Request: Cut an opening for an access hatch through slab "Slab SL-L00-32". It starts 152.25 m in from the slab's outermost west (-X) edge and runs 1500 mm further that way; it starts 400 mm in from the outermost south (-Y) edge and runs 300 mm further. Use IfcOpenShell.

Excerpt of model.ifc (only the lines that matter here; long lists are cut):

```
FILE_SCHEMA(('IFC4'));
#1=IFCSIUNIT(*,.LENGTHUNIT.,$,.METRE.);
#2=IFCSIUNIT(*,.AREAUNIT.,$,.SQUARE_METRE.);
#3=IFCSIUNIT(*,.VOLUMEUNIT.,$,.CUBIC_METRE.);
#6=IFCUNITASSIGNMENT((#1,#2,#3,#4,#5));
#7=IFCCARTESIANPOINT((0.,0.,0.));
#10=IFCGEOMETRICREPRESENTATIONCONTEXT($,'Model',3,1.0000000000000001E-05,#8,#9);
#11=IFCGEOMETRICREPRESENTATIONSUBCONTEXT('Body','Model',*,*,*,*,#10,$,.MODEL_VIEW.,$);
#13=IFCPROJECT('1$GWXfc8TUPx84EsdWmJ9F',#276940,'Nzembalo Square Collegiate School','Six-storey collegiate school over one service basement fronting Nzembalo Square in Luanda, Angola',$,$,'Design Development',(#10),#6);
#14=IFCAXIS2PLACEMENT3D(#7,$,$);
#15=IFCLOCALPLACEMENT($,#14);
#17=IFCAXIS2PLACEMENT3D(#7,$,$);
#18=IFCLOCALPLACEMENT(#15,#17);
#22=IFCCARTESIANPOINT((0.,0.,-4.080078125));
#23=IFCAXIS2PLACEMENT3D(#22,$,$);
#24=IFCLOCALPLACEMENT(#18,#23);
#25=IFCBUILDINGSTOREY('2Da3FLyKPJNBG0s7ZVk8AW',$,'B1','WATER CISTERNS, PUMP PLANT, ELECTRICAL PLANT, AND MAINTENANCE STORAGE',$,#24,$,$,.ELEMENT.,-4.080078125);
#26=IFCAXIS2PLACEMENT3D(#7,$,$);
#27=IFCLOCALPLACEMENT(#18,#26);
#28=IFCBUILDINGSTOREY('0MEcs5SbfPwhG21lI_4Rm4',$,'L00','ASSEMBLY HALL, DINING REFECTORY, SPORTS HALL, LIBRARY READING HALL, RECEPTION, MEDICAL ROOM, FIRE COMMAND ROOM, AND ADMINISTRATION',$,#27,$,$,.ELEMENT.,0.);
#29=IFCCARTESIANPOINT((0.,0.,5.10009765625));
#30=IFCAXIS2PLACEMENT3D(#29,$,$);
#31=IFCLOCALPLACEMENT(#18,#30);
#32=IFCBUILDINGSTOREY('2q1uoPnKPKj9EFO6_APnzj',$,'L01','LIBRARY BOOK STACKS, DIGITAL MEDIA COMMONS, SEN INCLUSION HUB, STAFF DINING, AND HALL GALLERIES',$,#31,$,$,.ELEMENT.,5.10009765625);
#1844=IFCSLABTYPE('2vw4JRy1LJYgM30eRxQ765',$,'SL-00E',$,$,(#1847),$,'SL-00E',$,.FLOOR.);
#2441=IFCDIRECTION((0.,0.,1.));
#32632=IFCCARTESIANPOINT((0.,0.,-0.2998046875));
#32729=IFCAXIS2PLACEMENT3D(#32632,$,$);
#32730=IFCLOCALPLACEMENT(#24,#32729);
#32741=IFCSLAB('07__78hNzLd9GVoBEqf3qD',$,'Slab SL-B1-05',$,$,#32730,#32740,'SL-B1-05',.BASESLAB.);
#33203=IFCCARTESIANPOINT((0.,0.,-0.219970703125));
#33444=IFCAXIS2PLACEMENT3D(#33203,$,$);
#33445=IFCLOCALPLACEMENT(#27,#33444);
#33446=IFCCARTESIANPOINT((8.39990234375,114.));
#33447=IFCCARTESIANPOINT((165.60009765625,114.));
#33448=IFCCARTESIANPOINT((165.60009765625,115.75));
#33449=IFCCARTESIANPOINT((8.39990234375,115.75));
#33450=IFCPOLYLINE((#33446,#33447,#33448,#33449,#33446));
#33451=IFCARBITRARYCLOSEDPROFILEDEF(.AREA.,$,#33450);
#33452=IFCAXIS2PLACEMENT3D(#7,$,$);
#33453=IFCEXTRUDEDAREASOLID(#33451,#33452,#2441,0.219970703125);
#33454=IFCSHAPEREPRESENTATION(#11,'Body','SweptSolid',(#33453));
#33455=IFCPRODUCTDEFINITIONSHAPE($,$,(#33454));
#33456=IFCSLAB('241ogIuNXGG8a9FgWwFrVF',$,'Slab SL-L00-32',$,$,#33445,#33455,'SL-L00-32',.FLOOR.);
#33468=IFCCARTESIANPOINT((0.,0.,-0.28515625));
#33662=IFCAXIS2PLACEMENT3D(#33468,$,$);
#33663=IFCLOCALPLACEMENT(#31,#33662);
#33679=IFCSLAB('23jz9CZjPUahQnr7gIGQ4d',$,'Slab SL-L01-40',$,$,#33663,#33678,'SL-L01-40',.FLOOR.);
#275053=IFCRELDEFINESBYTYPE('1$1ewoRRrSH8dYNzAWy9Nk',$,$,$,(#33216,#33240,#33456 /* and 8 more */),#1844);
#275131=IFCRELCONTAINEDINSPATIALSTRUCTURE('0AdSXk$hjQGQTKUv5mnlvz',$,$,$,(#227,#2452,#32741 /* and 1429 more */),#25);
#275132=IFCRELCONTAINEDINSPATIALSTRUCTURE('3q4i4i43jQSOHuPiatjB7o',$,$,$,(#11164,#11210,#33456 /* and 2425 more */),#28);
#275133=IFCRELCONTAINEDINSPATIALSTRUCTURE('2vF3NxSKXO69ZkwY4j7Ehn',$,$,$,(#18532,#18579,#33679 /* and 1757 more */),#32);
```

```python
import numpy as np
import ifcopenshell
import ifcopenshell.api.feature
import ifcopenshell.api.geometry
import ifcopenshell.api.root
import ifcopenshell.geom
import ifcopenshell.util.placement
import ifcopenshell.util.representation
import ifcopenshell.util.shape
import ifcopenshell.util.unit

model = ifcopenshell.open("model.ifc")
unit_scale = ifcopenshell.util.unit.calculate_unit_scale(model)
settings = ifcopenshell.geom.settings()


def volume(element):
    """Net volume in cubic metres, openings subtracted."""
    shape = ifcopenshell.geom.create_shape(settings, element)
    return ifcopenshell.util.shape.get_volume(shape.geometry)


slab = model.by_guid("241ogIuNXGG8a9FgWwFrVF")
before = volume(slab)

# Extent in the slab's own axes, in metres. The edges named are its -X and -Y sides.
slab_shape = ifcopenshell.geom.create_shape(settings, slab)
vertices = ifcopenshell.util.shape.get_vertices(slab_shape.geometry)
x_min, y_min, bottom = vertices.min(axis=0)
top = vertices[:, 2].max()

opening = ifcopenshell.api.root.create_entity(model, ifc_class="IfcOpeningElement", name="Access hatch opening", predefined_type="OPENING")
context = ifcopenshell.util.representation.get_context(model, "Model", "Body", "MODEL_VIEW")
width, depth = 1.5, 0.3
outline = [(0.0, 0.0), (width, 0.0), (width, depth), (0.0, depth), (0.0, 0.0)]
# Overshoot both faces by 50 mm so the cut is clean.
shape = ifcopenshell.api.geometry.add_slab_representation(
    model, context=context, depth=top - bottom + 0.1, polyline=outline
)
ifcopenshell.api.geometry.assign_representation(model, product=opening, representation=shape)

matrix = ifcopenshell.util.placement.get_local_placement(slab.ObjectPlacement)
matrix[:, 3] = matrix @ np.append(np.array([x_min + 152.25, y_min + 0.4, bottom - 0.05]) / unit_scale, 1.0)
ifcopenshell.api.geometry.edit_object_placement(model, product=opening, matrix=matrix, is_si=False)
ifcopenshell.api.feature.add_feature(model, feature=opening, element=slab)

after = volume(slab)

print(f"slab volume {before:.3f} -> {after:.3f} m3")

model.write("model_edited.ifc")
```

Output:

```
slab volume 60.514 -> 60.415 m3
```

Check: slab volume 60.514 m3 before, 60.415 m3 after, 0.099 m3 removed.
